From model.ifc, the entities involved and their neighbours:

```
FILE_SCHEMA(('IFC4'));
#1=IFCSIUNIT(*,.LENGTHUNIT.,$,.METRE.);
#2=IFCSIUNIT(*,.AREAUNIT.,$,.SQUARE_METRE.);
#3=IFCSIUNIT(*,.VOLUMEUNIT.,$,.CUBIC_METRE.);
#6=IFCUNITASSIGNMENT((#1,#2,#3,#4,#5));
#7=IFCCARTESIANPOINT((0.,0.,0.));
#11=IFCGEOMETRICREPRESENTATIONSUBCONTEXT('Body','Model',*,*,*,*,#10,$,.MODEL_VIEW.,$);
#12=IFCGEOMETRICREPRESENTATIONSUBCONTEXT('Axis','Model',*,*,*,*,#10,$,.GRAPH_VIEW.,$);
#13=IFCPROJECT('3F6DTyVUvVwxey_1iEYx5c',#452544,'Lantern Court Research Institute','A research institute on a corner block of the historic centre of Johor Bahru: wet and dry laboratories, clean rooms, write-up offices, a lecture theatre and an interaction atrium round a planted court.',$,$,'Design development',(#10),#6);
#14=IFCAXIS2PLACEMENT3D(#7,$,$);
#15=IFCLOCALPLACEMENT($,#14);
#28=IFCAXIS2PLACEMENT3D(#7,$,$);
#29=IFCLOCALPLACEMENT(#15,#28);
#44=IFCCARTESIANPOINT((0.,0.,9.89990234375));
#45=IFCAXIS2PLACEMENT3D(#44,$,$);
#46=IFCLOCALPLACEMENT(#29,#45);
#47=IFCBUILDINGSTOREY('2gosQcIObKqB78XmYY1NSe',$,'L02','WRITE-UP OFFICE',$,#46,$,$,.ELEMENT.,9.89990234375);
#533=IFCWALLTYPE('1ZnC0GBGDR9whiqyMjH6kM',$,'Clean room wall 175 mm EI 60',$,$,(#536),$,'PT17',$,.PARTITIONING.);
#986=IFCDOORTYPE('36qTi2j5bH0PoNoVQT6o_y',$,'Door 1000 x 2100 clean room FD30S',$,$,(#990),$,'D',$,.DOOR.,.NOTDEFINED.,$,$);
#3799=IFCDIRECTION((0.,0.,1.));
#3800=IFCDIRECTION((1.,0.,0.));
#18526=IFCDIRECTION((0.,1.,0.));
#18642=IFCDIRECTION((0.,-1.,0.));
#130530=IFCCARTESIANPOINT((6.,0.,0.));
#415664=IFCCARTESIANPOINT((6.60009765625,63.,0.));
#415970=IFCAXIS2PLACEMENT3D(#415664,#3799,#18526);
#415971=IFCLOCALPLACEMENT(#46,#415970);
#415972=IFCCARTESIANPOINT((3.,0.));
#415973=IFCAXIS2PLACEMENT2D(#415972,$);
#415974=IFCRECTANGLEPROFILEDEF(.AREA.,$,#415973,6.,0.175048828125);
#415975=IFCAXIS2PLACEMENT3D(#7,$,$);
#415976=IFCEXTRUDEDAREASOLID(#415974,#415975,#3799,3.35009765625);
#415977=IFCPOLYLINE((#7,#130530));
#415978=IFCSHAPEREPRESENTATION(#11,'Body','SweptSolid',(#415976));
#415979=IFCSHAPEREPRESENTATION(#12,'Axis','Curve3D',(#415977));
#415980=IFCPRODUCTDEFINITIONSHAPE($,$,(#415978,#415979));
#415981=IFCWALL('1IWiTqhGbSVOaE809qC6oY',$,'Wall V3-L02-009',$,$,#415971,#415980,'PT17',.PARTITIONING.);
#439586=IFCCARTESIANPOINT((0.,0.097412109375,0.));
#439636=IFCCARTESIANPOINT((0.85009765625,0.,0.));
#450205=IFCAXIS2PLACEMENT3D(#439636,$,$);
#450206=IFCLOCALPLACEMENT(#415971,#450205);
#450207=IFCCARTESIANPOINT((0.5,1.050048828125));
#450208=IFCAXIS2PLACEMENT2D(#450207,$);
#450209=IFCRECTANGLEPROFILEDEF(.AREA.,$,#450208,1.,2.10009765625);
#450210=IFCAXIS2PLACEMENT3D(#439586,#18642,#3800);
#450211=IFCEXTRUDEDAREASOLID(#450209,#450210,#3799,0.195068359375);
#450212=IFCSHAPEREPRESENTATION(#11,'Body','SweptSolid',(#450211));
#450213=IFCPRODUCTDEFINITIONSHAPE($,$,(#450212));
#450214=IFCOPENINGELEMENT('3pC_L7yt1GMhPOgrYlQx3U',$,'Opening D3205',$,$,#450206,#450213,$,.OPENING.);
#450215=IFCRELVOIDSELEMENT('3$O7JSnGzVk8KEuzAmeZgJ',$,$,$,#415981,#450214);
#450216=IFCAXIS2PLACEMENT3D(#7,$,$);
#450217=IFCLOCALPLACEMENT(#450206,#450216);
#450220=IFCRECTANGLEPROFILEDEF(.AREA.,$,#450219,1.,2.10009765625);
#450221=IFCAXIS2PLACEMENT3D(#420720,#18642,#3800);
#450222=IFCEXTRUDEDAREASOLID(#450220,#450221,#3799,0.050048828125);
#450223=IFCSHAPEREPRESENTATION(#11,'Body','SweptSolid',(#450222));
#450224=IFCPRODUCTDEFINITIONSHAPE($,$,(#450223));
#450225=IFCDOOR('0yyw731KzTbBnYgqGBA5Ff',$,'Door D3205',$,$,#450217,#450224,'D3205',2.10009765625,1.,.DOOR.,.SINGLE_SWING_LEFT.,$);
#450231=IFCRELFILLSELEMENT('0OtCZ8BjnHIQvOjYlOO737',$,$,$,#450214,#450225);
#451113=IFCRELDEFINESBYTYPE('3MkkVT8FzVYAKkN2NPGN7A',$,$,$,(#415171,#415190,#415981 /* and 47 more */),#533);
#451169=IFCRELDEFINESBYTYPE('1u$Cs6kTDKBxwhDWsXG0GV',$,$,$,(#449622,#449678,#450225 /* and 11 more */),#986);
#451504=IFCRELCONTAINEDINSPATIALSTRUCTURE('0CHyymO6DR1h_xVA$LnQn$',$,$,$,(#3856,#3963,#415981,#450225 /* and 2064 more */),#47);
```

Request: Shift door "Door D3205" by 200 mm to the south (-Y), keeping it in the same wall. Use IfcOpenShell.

```python
import ifcopenshell
import ifcopenshell.api.geometry
import ifcopenshell.util.placement
import ifcopenshell.util.unit

model = ifcopenshell.open("model.ifc")
unit_scale = ifcopenshell.util.unit.calculate_unit_scale(model)

door = model.by_guid("0yyw731KzTbBnYgqGBA5Ff")
opening = door.FillsVoids[0].RelatingOpeningElement
wall = opening.VoidsElements[0].RelatingBuildingElement

wall_matrix = ifcopenshell.util.placement.get_local_placement(wall.ObjectPlacement)
shift = wall_matrix[:3, 0] * -0.2 / unit_scale
before = ifcopenshell.util.placement.get_local_placement(door.ObjectPlacement)[:3, 3].copy()

# The door is placed relative to its opening, so it follows when the opening moves.
matrix = ifcopenshell.util.placement.get_local_placement(opening.ObjectPlacement)
matrix[:3, 3] += shift
ifcopenshell.api.geometry.edit_object_placement(
    model, product=opening, matrix=matrix, is_si=False, should_transform_children=True
)

after = ifcopenshell.util.placement.get_local_placement(door.ObjectPlacement)[:3, 3]
print("door moved by", (after - before).round(3) + 0.0)

model.write("model_edited.ifc")
```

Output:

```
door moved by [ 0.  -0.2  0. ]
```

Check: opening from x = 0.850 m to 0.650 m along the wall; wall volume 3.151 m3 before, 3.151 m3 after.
